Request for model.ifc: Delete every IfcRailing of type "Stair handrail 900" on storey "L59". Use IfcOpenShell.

First a look at what the model holds.

```python
import ifcopenshell
import ifcopenshell.util.element

model = ifcopenshell.open("model.ifc")
print(model.schema)
storey = next(s for s in model.by_type("IfcBuildingStorey") if s.Name == "L59")
railings = [e for e in ifcopenshell.util.element.get_decomposition(storey) if e.is_a("IfcRailing")]
seen = {}
for e in railings:
    element_type = ifcopenshell.util.element.get_type(e)
    name = element_type.Name if element_type not in (None, e) else None
    seen[name] = seen.get(name, 0) + 1
for name, count in sorted(seen.items(), key=str):
    print(count, "x", name)
```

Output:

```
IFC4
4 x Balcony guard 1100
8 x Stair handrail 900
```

```python
import ifcopenshell
import ifcopenshell.api.root
import ifcopenshell.util.element

model = ifcopenshell.open("model.ifc")

storey = next(s for s in model.by_type("IfcBuildingStorey") if s.Name == "L59")
railings = [e for e in ifcopenshell.util.element.get_decomposition(storey) if e.is_a("IfcRailing")]
targets = [e for e in railings if (t := ifcopenshell.util.element.get_type(e)) not in (None, e) and t.Name == "Stair handrail 900"]

for e in targets:
    ifcopenshell.api.root.remove_product(model, product=e)
print(len(targets), "removed")

model.write("model_edited.ifc")
```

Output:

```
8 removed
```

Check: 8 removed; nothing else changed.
